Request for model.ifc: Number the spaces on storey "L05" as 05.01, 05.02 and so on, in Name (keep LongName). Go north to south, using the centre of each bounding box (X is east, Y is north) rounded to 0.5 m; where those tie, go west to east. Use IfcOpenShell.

First a look at what the model holds.

```python
import ifcopenshell
import ifcopenshell.util.element
import ifcopenshell.util.placement

model = ifcopenshell.open("model.ifc")
print(model.schema)
storey = next(s for s in model.by_type("IfcBuildingStorey") if s.Name == "L05")
spaces = [e for e in ifcopenshell.util.element.get_decomposition(storey) if e.is_a("IfcSpace")]
for e in sorted(spaces, key=lambda e: e.id()):
    origin = ifcopenshell.util.placement.get_local_placement(e.ObjectPlacement)[:3, 3]
    print(e.id(), e.Name, e.LongName, origin.round(2) + 0.0, sep=" | ")
```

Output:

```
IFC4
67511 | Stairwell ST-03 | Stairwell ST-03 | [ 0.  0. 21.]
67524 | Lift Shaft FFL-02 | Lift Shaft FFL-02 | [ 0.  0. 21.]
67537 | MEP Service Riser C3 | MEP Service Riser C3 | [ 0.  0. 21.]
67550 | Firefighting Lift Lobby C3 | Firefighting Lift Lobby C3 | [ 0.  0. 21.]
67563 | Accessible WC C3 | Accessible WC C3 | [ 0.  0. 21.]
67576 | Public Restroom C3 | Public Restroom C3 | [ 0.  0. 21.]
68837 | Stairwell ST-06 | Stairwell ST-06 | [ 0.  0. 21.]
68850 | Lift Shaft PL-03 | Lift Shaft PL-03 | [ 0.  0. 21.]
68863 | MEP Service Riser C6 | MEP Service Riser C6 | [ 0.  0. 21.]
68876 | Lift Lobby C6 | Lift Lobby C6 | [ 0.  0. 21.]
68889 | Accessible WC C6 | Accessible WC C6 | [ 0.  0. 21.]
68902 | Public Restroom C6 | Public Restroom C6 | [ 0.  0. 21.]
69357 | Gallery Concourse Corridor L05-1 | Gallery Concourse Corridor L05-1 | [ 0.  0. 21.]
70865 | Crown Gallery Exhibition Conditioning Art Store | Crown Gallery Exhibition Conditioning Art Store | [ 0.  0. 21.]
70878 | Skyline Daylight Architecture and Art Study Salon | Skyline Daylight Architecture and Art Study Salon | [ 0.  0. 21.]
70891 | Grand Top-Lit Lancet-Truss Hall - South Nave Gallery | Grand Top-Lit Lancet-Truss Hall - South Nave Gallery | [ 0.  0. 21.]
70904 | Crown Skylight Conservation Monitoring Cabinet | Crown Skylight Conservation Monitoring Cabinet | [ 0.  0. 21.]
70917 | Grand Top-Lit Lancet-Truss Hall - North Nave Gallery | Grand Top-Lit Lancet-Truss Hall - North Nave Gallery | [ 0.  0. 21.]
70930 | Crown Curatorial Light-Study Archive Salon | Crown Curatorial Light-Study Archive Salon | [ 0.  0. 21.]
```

```python
import ifcopenshell
import ifcopenshell.geom
import ifcopenshell.util.element
import ifcopenshell.util.shape

model = ifcopenshell.open("model.ifc")
settings = ifcopenshell.geom.settings()
settings.set("use-world-coords", True)


def centre(element):
    shape = ifcopenshell.geom.create_shape(settings, element)
    return ifcopenshell.util.shape.get_bbox_centroid(shape.geometry)


storey = next(s for s in model.by_type("IfcBuildingStorey") if s.Name == "L05")
spaces = [e for e in ifcopenshell.util.element.get_decomposition(storey) if e.is_a("IfcSpace")]

# Insertion points can sit at a corner or the storey origin, so sort by the geometry (in metres).
centres = {e: centre(e) for e in spaces}
spaces.sort(key=lambda e: (-round(centres[e][1] / 0.5), centres[e][0]))

for i, e in enumerate(spaces, start=1):
    number = f"05.{i:02d}"
    e.Name = number
    print(e.id(), number)

model.write("model-out.ifc")
```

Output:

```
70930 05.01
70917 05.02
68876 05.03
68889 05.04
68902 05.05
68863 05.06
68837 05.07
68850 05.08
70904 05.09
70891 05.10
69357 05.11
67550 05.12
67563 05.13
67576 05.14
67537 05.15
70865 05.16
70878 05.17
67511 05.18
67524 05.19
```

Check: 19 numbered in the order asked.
